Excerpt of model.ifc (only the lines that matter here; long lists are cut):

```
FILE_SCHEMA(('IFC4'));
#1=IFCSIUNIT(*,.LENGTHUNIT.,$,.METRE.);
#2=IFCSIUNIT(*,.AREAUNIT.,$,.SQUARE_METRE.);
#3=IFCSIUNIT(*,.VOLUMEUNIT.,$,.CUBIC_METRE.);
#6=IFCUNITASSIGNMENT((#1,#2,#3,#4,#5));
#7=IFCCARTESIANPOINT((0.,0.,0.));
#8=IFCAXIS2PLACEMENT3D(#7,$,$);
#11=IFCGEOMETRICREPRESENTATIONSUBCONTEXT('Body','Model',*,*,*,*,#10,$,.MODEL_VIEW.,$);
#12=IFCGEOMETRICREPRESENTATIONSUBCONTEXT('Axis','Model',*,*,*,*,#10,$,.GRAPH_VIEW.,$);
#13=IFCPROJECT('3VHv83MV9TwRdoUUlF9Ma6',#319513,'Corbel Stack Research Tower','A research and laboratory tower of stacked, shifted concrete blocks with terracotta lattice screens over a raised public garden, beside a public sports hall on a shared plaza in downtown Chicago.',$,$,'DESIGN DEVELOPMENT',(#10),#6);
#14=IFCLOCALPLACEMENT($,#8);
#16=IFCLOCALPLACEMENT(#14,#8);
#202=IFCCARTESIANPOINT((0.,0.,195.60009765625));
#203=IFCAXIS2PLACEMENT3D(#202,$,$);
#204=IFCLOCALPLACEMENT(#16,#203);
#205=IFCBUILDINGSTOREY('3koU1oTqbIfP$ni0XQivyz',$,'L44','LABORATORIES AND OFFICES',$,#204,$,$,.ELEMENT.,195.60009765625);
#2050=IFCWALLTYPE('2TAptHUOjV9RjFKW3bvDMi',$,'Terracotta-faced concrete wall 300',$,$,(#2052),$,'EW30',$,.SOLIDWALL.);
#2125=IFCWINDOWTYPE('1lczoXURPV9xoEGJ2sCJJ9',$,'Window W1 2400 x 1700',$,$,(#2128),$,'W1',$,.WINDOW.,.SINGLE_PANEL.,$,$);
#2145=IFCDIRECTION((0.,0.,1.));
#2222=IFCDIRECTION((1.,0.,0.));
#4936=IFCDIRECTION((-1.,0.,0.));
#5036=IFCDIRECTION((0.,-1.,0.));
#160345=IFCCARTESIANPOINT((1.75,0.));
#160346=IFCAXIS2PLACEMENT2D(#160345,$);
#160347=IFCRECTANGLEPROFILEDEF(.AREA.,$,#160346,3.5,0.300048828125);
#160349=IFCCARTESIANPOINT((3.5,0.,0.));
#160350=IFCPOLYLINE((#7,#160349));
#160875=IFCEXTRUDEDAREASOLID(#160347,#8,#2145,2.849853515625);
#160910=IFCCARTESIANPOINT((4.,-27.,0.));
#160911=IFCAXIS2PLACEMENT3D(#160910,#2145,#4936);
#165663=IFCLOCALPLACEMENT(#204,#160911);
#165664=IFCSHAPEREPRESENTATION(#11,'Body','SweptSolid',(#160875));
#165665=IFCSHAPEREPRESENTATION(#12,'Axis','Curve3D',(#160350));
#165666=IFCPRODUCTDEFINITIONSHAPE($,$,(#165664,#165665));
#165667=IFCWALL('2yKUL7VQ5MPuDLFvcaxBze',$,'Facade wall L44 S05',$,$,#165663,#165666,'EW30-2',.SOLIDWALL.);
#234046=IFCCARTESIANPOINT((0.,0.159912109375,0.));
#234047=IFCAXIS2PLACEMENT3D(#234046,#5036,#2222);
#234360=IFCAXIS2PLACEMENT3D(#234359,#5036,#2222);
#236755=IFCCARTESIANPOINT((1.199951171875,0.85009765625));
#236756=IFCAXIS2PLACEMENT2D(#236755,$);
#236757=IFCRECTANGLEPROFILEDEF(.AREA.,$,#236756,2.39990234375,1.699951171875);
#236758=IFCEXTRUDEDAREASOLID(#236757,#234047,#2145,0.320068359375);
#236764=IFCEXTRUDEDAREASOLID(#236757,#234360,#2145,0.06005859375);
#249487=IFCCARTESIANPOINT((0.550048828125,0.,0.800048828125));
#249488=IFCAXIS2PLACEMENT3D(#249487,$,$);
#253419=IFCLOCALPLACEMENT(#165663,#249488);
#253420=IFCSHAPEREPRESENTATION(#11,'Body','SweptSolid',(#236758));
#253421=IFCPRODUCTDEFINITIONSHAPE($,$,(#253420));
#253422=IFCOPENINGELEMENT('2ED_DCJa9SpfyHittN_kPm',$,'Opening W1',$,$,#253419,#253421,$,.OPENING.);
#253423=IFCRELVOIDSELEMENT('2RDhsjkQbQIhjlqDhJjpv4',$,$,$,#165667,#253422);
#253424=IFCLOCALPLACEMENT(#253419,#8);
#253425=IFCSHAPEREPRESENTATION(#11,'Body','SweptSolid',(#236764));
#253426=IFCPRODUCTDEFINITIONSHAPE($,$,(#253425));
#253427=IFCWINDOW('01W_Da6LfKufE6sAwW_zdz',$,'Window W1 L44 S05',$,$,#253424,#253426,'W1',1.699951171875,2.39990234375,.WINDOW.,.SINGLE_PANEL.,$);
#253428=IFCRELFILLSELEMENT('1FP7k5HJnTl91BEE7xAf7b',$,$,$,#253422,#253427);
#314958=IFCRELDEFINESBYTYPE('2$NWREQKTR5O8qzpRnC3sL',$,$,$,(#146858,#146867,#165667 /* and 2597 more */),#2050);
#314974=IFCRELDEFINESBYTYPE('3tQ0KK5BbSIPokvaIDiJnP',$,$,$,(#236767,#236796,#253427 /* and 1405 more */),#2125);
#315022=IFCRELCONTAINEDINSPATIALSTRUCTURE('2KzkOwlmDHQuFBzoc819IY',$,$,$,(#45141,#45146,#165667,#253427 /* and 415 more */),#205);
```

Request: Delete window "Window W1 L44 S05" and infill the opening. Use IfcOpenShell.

```python
import ifcopenshell
import ifcopenshell.api.feature
import ifcopenshell.api.root
import ifcopenshell.geom
import ifcopenshell.util.shape

model = ifcopenshell.open("model.ifc")
settings = ifcopenshell.geom.settings()


def volume(element):
    """Net volume in cubic metres, openings subtracted."""
    shape = ifcopenshell.geom.create_shape(settings, element)
    return ifcopenshell.util.shape.get_volume(shape.geometry)


window = model.by_id(253427)
opening = window.FillsVoids[0].RelatingOpeningElement
wall = opening.VoidsElements[0].RelatingBuildingElement
before = volume(wall)

ifcopenshell.api.root.remove_product(model, product=window)
ifcopenshell.api.feature.remove_feature(model, feature=opening)

after = volume(wall)

print(f"wall volume {before:.3f} -> {after:.3f} m3")

model.write("model_edited.ifc")
```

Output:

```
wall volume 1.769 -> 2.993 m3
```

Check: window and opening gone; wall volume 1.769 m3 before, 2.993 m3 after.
